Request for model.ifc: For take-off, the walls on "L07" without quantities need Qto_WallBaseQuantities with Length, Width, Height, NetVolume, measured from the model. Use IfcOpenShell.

First a look at what the model holds.

```python
import ifcopenshell
import ifcopenshell.util.element
import ifcopenshell.util.unit

model = ifcopenshell.open("model.ifc")
print(model.schema)
for unit_type in ("LENGTHUNIT", "AREAUNIT", "VOLUMEUNIT"):
    print(unit_type, ifcopenshell.util.unit.calculate_unit_scale(model, unit_type))
storey = next(s for s in model.by_type("IfcBuildingStorey") if s.Name == "L07")
walls = [e for e in ifcopenshell.util.element.get_decomposition(storey) if e.is_a("IfcWall")]
for e in sorted(walls, key=lambda e: e.id()):
    print(e.id(), e.is_a(), e.Name, list(ifcopenshell.util.element.get_psets(e, qtos_only=True)), sep=" | ")
```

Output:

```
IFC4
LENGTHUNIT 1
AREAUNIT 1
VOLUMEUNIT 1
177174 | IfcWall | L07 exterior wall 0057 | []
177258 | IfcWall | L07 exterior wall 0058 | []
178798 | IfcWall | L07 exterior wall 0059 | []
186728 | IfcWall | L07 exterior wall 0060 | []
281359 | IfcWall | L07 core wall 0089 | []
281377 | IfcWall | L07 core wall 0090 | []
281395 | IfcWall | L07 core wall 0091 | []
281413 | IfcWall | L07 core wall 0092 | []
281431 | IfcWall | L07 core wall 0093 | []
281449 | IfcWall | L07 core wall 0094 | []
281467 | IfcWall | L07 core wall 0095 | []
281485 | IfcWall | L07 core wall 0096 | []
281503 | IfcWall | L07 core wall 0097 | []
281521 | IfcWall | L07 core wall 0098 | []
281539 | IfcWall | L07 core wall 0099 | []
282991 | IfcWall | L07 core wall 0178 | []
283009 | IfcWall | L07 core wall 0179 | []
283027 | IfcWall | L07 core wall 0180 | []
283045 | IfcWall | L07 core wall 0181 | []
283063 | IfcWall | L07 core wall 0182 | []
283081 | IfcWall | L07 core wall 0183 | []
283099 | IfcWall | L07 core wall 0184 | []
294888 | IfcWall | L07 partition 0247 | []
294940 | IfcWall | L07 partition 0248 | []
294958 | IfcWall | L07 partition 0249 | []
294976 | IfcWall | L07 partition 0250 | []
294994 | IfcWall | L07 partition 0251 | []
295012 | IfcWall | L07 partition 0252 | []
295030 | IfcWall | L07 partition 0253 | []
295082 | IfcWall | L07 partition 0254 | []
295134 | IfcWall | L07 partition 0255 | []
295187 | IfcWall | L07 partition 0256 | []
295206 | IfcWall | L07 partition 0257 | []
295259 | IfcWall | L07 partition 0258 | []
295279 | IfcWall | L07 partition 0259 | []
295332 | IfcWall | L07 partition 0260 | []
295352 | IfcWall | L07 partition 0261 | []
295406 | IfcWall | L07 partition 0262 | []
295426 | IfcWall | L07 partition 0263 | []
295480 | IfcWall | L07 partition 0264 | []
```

```python
import ifcopenshell
import ifcopenshell.api.pset
import ifcopenshell.geom
import ifcopenshell.util.element
import ifcopenshell.util.shape
import ifcopenshell.util.unit

model = ifcopenshell.open("model.ifc")
unit_scale = ifcopenshell.util.unit.calculate_unit_scale(model)
volume_scale = ifcopenshell.util.unit.calculate_unit_scale(model, "VOLUMEUNIT")
settings = ifcopenshell.geom.settings()

storey = next(s for s in model.by_type("IfcBuildingStorey") if s.Name == "L07")
walls = [e for e in ifcopenshell.util.element.get_decomposition(storey) if e.is_a("IfcWall")]

for e in sorted(walls, key=lambda e: e.id()):
    if ifcopenshell.util.element.get_psets(e, qtos_only=True, should_inherit=False):
        continue
    # Geometry comes back in metres, in the element's own axes.
    shape = ifcopenshell.geom.create_shape(settings, e)
    values = {
        "Length": ifcopenshell.util.shape.get_x(shape.geometry) / unit_scale,
        "Width": ifcopenshell.util.shape.get_y(shape.geometry) / unit_scale,
        "Height": ifcopenshell.util.shape.get_z(shape.geometry) / unit_scale,
        "NetVolume": ifcopenshell.util.shape.get_volume(shape.geometry) / volume_scale,
    }
    qto = ifcopenshell.api.pset.add_qto(model, product=e, name="Qto_WallBaseQuantities")
    ifcopenshell.api.pset.edit_qto(model, qto=qto, properties=values)
    print(e.id(), {k: round(v, 3) for k, v in values.items()})

model.write("model_rev.ifc")
```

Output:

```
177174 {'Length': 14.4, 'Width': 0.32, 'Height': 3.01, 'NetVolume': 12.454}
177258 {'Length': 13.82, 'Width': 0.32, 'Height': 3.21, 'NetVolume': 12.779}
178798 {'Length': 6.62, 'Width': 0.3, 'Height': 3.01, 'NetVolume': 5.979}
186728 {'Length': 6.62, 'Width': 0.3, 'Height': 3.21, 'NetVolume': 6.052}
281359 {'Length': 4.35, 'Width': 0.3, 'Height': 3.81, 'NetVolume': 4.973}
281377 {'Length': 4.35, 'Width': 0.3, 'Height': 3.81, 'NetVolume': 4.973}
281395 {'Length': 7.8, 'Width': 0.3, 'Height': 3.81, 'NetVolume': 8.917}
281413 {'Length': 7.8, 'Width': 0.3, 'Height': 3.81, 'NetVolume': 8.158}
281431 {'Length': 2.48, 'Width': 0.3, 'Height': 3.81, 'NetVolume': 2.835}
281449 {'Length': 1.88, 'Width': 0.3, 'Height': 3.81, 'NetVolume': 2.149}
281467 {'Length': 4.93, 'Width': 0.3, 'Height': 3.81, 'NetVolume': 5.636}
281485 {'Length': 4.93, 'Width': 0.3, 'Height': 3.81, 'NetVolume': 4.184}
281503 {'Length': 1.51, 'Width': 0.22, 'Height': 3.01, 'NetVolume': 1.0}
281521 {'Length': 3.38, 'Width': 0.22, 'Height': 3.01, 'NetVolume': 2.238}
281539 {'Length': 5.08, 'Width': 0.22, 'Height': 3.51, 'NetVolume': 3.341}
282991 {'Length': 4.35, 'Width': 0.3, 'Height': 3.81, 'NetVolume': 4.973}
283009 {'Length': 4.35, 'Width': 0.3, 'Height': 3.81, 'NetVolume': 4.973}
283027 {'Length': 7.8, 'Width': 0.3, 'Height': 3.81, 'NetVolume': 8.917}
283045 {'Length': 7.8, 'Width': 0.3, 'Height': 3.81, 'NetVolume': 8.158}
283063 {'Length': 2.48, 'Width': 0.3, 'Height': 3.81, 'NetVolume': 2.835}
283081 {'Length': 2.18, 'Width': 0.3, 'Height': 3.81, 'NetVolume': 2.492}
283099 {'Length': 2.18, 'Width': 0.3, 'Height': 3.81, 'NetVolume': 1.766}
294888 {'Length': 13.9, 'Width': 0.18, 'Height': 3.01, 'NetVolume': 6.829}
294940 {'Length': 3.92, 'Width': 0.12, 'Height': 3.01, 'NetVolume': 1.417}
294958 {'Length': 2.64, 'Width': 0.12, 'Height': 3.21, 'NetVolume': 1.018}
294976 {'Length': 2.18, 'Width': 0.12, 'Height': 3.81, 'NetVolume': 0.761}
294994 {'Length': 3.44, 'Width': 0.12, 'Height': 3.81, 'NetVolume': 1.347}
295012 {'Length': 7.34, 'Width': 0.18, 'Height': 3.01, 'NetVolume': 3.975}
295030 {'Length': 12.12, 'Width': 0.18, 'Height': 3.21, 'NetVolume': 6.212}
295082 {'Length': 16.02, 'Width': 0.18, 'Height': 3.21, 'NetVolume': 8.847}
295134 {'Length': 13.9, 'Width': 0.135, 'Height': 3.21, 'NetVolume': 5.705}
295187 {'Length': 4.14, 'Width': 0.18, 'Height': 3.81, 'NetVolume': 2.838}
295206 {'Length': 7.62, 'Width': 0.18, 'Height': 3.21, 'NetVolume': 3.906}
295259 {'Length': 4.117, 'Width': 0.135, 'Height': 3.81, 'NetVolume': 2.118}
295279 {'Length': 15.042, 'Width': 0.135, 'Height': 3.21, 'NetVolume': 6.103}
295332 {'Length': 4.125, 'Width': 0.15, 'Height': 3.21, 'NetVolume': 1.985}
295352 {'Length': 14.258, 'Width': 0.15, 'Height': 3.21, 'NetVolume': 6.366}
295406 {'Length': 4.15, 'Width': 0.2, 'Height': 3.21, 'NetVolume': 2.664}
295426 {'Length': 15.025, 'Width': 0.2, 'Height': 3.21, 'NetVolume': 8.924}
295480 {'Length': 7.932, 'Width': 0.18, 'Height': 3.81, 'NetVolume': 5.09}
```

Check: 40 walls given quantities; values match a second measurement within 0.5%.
